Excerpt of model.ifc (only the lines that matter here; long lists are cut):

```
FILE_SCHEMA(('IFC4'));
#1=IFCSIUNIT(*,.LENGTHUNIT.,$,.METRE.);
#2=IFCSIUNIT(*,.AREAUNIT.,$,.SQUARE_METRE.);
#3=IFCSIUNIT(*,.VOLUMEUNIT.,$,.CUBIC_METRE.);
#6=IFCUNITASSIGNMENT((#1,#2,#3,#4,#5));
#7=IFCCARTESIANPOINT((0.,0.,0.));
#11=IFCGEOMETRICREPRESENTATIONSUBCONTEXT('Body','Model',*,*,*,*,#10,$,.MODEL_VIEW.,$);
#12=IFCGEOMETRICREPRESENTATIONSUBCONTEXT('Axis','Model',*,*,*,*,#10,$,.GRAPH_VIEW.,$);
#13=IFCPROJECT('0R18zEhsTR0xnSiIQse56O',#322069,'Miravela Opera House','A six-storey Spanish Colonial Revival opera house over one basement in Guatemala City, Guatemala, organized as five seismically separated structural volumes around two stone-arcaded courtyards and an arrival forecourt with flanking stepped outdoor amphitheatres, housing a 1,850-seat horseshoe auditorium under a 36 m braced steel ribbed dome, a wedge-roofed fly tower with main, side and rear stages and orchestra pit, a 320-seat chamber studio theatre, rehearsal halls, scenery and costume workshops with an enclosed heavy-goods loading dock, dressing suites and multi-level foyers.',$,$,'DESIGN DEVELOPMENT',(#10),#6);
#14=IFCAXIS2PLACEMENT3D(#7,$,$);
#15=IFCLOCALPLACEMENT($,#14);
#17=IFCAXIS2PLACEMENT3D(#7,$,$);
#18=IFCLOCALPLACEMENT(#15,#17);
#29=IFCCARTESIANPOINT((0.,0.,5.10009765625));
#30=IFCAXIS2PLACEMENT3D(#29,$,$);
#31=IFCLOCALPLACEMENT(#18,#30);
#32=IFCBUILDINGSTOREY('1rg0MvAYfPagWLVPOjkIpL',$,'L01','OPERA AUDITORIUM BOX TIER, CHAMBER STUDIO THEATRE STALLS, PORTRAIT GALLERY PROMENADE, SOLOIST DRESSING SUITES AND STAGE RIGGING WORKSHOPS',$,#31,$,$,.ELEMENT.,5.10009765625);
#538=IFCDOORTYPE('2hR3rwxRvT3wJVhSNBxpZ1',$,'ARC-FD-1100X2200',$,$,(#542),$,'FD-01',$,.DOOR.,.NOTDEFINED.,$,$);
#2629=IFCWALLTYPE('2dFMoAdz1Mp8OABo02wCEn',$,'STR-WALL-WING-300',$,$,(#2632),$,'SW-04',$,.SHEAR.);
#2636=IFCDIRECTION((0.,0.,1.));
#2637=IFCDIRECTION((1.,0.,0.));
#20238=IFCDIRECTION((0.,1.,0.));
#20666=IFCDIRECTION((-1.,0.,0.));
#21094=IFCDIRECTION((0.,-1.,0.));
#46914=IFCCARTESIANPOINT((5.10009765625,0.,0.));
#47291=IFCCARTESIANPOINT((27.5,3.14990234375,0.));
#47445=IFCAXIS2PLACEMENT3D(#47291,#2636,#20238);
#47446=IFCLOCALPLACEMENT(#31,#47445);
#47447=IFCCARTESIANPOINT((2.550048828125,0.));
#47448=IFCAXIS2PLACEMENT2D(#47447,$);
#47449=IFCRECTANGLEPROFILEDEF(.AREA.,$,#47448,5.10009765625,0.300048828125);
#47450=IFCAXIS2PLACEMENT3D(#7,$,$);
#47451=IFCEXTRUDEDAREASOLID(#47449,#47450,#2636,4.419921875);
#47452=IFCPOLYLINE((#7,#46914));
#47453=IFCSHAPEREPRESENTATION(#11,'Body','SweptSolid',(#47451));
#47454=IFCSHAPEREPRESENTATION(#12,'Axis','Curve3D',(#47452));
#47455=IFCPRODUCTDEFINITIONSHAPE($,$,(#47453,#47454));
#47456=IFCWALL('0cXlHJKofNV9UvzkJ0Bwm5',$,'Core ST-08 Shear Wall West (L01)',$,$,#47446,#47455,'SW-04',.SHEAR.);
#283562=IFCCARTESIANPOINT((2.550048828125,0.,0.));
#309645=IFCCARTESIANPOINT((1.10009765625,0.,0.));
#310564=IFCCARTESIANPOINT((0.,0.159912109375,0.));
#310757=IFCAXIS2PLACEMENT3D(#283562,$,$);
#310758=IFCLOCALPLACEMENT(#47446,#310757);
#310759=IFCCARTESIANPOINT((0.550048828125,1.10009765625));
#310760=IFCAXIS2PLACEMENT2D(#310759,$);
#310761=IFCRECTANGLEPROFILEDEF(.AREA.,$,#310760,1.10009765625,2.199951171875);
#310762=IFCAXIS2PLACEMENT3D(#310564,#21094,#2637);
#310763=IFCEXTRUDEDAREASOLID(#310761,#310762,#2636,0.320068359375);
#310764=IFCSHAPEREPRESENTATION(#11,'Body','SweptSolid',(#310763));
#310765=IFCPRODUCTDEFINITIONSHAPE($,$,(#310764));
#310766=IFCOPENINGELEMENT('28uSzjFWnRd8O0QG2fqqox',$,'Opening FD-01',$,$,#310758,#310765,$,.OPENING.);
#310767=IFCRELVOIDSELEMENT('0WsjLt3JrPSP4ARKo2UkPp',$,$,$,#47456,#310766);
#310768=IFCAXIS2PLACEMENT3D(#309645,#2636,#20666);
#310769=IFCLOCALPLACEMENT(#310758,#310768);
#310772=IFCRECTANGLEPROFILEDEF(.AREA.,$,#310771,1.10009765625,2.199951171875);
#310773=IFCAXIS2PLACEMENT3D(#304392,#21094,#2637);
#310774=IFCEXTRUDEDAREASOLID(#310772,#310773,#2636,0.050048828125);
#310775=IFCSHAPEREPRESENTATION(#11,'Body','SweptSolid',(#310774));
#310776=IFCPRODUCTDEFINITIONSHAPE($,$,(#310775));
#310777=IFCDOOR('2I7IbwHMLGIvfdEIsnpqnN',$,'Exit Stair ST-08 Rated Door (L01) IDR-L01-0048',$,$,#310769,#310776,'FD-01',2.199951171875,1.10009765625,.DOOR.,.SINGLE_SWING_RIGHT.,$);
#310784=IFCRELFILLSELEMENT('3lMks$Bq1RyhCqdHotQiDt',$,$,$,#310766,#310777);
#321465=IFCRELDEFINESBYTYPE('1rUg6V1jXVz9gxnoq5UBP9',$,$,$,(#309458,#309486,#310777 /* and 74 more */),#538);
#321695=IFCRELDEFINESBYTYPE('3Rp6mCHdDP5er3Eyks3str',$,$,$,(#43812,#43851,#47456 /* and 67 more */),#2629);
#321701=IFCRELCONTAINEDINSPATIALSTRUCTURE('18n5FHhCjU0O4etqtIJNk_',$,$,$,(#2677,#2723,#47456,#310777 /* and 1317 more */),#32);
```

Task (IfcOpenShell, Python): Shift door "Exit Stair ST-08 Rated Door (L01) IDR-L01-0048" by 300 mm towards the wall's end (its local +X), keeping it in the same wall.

```python
import ifcopenshell
import ifcopenshell.api.geometry
import ifcopenshell.util.placement
import ifcopenshell.util.unit

model = ifcopenshell.open("model.ifc")
unit_scale = ifcopenshell.util.unit.calculate_unit_scale(model)

door = model.by_guid("2I7IbwHMLGIvfdEIsnpqnN")
opening = door.FillsVoids[0].RelatingOpeningElement
wall = opening.VoidsElements[0].RelatingBuildingElement

wall_matrix = ifcopenshell.util.placement.get_local_placement(wall.ObjectPlacement)
shift = wall_matrix[:3, 0] * 0.3 / unit_scale
before = ifcopenshell.util.placement.get_local_placement(door.ObjectPlacement)[:3, 3].copy()

# The door is placed relative to its opening, so it follows when the opening moves.
matrix = ifcopenshell.util.placement.get_local_placement(opening.ObjectPlacement)
matrix[:3, 3] += shift
ifcopenshell.api.geometry.edit_object_placement(
    model, product=opening, matrix=matrix, is_si=False, should_transform_children=True
)

after = ifcopenshell.util.placement.get_local_placement(door.ObjectPlacement)[:3, 3]
print("door moved by", (after - before).round(3) + 0.0)

model.write("model_v2.ifc")
```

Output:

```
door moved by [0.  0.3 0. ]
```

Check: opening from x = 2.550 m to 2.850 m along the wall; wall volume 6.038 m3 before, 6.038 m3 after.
